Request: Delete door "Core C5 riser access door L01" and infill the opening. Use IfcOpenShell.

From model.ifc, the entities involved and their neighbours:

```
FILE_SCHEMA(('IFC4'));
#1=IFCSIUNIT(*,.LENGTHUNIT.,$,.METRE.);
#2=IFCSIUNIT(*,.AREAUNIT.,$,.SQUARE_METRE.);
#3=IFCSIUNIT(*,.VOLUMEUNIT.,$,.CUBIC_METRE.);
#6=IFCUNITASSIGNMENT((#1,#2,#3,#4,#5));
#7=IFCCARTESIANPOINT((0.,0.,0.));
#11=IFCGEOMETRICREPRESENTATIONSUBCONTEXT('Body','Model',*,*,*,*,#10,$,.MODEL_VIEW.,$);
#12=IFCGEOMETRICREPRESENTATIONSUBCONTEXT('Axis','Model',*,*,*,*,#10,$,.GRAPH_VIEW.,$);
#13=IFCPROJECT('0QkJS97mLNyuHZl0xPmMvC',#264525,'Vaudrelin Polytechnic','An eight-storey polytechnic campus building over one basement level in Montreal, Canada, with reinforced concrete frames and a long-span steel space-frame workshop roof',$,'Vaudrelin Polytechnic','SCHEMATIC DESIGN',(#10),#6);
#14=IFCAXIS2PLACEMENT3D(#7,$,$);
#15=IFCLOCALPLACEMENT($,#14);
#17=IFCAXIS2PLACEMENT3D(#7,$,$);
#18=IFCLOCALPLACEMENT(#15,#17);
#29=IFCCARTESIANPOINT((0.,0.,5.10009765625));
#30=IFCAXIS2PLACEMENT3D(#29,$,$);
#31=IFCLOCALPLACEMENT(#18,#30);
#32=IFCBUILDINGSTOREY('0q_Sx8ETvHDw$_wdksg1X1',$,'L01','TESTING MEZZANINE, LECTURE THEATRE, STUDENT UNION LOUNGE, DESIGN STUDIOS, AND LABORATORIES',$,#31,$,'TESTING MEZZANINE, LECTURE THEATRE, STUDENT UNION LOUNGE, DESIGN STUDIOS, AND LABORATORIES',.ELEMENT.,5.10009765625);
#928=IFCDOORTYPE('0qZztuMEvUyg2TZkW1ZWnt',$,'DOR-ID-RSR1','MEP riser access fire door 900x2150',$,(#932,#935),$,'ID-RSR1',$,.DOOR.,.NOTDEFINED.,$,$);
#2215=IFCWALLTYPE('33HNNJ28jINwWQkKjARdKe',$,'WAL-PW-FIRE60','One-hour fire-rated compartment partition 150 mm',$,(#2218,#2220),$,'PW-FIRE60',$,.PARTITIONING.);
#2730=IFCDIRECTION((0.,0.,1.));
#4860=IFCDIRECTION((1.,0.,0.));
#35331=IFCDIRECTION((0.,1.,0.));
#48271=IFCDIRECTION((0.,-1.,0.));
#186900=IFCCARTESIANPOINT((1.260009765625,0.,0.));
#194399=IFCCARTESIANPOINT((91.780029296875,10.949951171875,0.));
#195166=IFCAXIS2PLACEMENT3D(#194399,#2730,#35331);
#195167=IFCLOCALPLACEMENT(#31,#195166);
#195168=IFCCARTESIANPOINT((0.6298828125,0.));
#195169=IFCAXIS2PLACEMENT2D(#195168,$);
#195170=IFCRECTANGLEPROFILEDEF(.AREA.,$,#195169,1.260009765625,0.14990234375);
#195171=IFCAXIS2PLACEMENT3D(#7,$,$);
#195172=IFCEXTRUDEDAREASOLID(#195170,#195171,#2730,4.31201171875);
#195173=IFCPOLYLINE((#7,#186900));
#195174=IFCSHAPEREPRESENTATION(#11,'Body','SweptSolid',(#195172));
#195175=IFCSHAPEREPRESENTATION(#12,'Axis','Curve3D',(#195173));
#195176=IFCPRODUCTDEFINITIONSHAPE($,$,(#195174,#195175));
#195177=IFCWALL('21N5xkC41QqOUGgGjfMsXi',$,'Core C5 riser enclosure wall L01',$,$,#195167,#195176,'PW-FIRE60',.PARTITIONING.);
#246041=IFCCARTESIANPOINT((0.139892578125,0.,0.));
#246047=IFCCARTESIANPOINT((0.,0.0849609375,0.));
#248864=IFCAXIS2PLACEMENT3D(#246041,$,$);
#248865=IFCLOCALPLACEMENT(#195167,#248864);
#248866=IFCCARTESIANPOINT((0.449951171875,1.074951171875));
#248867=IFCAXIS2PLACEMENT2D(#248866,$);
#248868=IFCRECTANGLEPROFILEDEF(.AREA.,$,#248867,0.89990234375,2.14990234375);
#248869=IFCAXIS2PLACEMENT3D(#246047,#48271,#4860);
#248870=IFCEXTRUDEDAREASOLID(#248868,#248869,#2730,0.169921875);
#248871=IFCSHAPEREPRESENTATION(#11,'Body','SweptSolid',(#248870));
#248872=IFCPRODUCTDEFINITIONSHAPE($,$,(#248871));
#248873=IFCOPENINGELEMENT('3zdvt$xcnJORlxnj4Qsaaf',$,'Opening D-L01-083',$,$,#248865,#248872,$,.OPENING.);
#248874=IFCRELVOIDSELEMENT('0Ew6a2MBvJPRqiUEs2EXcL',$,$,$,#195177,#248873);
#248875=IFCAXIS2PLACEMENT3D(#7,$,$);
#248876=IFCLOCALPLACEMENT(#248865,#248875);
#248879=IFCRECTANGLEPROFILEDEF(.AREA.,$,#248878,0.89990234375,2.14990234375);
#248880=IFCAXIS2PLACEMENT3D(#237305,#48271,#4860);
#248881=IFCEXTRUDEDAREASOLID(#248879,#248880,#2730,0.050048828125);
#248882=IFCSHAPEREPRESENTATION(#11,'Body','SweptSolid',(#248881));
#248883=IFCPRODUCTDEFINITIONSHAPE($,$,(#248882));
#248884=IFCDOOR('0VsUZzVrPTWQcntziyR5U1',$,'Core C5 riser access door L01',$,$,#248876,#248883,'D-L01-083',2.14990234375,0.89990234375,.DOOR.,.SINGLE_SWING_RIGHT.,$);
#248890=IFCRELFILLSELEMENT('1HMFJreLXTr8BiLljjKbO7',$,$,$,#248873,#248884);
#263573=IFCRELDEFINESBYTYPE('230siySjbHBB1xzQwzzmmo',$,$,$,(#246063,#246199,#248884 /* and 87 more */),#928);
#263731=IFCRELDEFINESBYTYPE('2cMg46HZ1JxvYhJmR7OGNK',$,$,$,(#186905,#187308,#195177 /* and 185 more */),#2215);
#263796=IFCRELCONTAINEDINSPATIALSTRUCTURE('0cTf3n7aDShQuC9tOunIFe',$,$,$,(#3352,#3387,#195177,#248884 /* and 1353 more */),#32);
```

```python
import ifcopenshell
import ifcopenshell.api.feature
import ifcopenshell.api.root
import ifcopenshell.geom
import ifcopenshell.util.shape

model = ifcopenshell.open("model.ifc")
settings = ifcopenshell.geom.settings()


def volume(element):
    """Net volume in cubic metres, openings subtracted."""
    shape = ifcopenshell.geom.create_shape(settings, element)
    return ifcopenshell.util.shape.get_volume(shape.geometry)


door = model.by_guid("0VsUZzVrPTWQcntziyR5U1")
opening = door.FillsVoids[0].RelatingOpeningElement
wall = opening.VoidsElements[0].RelatingBuildingElement
before = volume(wall)

ifcopenshell.api.root.remove_product(model, product=door)
ifcopenshell.api.feature.remove_feature(model, feature=opening)

after = volume(wall)

print(f"wall volume {before:.3f} -> {after:.3f} m3")

model.write("model_v2.ifc")
```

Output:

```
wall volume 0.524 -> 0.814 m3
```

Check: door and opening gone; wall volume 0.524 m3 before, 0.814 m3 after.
